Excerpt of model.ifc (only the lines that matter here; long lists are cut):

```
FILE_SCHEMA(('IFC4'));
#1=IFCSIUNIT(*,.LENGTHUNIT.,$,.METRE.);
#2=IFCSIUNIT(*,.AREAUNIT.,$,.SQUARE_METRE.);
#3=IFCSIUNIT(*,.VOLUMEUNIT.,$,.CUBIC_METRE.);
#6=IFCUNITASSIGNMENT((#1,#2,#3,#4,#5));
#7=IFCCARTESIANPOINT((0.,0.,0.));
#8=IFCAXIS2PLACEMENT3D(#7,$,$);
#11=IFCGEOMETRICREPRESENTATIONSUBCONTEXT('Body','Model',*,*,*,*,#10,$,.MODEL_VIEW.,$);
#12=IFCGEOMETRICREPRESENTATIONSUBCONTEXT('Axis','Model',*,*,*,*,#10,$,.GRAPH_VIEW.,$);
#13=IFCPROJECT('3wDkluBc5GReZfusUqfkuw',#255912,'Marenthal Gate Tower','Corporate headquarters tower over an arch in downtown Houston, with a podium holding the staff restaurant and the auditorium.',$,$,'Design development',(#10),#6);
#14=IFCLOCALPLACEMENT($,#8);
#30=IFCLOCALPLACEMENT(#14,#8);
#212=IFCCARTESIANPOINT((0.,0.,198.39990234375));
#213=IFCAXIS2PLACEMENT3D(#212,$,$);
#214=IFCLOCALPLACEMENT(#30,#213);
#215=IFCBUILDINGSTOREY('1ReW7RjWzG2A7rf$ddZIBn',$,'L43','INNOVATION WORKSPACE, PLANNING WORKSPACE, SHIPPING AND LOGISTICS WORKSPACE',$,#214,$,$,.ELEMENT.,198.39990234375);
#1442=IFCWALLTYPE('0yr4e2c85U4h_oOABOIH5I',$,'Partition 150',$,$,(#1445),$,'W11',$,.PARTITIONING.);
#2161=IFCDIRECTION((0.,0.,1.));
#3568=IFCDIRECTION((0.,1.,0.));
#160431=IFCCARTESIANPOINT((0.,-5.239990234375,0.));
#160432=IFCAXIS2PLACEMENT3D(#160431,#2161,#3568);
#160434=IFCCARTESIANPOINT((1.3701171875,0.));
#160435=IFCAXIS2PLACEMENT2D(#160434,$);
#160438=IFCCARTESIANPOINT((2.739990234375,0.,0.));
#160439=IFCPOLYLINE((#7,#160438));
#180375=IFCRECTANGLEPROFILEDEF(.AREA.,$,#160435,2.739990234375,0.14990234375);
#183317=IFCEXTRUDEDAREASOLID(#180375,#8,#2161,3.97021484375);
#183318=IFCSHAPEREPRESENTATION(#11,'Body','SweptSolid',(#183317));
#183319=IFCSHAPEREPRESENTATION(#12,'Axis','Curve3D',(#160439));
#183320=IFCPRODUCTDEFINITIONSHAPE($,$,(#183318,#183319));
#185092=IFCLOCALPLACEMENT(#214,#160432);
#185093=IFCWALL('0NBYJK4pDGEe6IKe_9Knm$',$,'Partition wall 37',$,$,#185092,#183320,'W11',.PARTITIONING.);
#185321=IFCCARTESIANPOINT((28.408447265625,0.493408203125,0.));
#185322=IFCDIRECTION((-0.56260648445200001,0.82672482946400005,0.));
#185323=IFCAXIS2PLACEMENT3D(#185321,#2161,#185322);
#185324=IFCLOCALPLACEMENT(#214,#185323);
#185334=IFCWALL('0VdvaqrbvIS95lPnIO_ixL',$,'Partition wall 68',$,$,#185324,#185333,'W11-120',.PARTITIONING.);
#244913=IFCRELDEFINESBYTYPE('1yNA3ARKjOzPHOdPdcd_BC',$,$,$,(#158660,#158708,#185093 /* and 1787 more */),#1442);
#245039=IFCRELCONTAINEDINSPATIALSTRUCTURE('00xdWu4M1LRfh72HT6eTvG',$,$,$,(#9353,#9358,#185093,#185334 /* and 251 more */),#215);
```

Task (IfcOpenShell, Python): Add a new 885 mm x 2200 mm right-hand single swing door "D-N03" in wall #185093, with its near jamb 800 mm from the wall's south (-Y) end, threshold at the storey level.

```python
import numpy as np
import ifcopenshell
import ifcopenshell.api.feature
import ifcopenshell.api.geometry
import ifcopenshell.api.root
import ifcopenshell.api.spatial
import ifcopenshell.geom
import ifcopenshell.util.element
import ifcopenshell.util.placement
import ifcopenshell.util.representation
import ifcopenshell.util.shape
import ifcopenshell.util.unit

model = ifcopenshell.open("model.ifc")
unit_scale = ifcopenshell.util.unit.calculate_unit_scale(model)
settings = ifcopenshell.geom.settings()


def volume(element):
    """Net volume in cubic metres, openings subtracted."""
    shape = ifcopenshell.geom.create_shape(settings, element)
    return ifcopenshell.util.shape.get_volume(shape.geometry)


wall = model.by_id(185093)
storey = ifcopenshell.util.element.get_container(wall, ifc_class="IfcBuildingStorey")
context = ifcopenshell.util.representation.get_context(model, "Model", "Body", "MODEL_VIEW")
before = volume(wall)

width, height, from_end, sill = 0.885, 2.2, 0.8, 0.0  # metres

# The wall runs along its own X axis, and the end named is its -X end.
wall_shape = ifcopenshell.geom.create_shape(settings, wall)
x, y, z = ifcopenshell.util.shape.get_vertices(wall_shape.geometry).T
start = x.min() + from_end
face, thickness = float(y.min()), float(y.max() - y.min())
wall_matrix = ifcopenshell.util.placement.get_local_placement(wall.ObjectPlacement)
level = ifcopenshell.util.placement.get_local_placement(storey.ObjectPlacement)[2, 3]


def in_wall(x, y):
    """Placement at x, y metres in the wall's axes, at sill height."""
    matrix = wall_matrix.copy()
    matrix[:, 3] = wall_matrix @ np.array([x / unit_scale, y / unit_scale, 0.0, 1.0])
    matrix[2, 3] = level + sill / unit_scale
    return matrix


# Opening: a box that overshoots both wall faces by 50 mm.
opening = ifcopenshell.api.root.create_entity(model, ifc_class="IfcOpeningElement", predefined_type="OPENING")
box = ifcopenshell.api.geometry.add_wall_representation(
    model, context=context, length=width, height=height, thickness=thickness + 0.1
)
ifcopenshell.api.geometry.assign_representation(model, product=opening, representation=box)
ifcopenshell.api.geometry.edit_object_placement(model, product=opening, matrix=in_wall(start, face - 0.05), is_si=False)
ifcopenshell.api.feature.add_feature(model, feature=opening, element=wall)

door = ifcopenshell.api.root.create_entity(model, ifc_class="IfcDoor", name="D-N03", predefined_type="DOOR")
door.OverallWidth, door.OverallHeight = width / unit_scale, height / unit_scale
door.OperationType = "SINGLE_SWING_RIGHT"
body = ifcopenshell.api.geometry.add_door_representation(
    model,
    context=context,
    overall_width=door.OverallWidth,
    overall_height=door.OverallHeight,
    operation_type="SINGLE_SWING_RIGHT",
    lining_properties={"LiningDepth": thickness / unit_scale, "ThresholdDepth": thickness / unit_scale},
)
ifcopenshell.api.geometry.assign_representation(model, product=door, representation=body)
ifcopenshell.api.spatial.assign_container(model, products=[door], relating_structure=storey)
ifcopenshell.api.feature.add_filling(model, opening=opening, element=door)

# The lining spans the wall, so the door starts at the wall face.
ifcopenshell.api.geometry.edit_object_placement(model, product=door, matrix=in_wall(start, face), is_si=False)

after = volume(wall)

print(f"wall volume {before:.3f} -> {after:.3f} m3")

model.write("model_v2.ifc")
```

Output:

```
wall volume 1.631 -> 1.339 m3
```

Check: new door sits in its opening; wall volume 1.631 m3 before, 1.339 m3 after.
